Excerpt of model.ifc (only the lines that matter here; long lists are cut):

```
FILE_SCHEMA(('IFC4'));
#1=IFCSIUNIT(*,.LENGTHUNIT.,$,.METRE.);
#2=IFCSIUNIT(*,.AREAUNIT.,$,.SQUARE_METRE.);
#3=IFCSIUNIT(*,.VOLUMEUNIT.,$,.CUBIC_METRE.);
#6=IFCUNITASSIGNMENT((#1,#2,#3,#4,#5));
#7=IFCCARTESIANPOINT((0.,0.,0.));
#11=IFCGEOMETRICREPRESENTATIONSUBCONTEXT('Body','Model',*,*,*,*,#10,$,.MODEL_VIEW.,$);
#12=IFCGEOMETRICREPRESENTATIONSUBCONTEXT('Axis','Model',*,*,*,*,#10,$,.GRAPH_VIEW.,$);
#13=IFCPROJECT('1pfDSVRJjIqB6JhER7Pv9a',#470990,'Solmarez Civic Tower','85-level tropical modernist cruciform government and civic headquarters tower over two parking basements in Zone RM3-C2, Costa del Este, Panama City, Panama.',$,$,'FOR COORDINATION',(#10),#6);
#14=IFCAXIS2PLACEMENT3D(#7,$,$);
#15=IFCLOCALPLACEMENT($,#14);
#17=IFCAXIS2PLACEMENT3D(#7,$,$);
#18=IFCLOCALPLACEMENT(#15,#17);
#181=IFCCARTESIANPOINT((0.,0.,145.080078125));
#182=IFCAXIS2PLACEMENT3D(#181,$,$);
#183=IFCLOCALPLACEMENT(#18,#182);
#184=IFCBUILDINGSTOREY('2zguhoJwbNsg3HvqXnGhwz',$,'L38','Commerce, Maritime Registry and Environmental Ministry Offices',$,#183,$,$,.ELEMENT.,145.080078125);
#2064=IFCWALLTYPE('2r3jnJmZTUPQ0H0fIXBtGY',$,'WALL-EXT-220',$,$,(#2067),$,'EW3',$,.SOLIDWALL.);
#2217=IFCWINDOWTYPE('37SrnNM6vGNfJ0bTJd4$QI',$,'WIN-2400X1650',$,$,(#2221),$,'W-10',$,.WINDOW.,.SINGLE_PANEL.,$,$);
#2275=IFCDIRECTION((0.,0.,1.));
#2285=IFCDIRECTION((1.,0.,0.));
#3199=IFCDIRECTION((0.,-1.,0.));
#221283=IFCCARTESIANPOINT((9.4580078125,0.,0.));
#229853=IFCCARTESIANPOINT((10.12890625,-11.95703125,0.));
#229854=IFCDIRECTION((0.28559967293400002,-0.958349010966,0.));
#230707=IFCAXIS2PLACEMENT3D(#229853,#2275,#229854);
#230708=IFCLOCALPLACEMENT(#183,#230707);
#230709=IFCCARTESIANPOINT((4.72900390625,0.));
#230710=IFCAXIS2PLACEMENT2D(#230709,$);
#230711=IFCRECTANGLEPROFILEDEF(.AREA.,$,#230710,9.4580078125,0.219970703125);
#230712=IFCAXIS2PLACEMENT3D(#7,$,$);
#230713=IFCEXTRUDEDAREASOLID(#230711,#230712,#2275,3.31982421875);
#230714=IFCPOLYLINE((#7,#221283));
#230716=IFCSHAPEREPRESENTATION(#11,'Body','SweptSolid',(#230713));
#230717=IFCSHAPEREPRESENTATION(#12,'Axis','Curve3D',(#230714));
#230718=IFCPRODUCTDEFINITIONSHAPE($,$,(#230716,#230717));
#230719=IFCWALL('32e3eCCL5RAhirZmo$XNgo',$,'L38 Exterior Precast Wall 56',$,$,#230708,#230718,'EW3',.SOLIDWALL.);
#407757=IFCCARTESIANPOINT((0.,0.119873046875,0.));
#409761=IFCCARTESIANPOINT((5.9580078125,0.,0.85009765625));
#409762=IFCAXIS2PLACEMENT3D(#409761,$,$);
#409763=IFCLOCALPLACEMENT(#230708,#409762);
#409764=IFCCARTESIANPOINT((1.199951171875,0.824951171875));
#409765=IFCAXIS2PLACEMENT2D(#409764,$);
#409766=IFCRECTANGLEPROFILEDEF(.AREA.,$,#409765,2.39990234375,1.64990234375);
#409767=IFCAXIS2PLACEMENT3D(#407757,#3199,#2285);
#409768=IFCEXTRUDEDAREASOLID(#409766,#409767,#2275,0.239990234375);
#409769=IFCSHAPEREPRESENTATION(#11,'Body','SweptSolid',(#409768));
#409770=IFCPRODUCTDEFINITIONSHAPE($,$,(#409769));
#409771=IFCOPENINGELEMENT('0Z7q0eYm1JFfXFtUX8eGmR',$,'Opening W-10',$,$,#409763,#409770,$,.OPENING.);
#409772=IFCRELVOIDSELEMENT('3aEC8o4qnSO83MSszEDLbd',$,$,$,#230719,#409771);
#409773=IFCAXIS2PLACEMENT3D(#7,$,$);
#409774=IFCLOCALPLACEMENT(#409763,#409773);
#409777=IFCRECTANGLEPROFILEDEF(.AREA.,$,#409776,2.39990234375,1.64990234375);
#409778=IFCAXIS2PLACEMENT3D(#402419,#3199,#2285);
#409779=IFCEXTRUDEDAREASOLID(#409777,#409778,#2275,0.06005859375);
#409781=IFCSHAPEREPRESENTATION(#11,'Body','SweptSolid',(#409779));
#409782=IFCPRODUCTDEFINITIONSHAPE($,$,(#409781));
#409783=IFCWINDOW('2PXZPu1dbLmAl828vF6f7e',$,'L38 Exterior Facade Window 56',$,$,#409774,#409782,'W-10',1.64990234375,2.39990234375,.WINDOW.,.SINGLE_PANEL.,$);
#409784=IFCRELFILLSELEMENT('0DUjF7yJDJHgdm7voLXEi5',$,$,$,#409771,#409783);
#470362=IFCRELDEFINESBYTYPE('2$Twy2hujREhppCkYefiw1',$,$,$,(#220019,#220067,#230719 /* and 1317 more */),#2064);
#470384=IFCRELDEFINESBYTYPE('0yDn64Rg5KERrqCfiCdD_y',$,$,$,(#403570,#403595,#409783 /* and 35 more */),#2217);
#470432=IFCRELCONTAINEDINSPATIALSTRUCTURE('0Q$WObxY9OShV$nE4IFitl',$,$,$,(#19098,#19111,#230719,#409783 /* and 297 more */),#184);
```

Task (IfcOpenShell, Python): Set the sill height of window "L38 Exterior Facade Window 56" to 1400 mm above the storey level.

```python
import numpy as np
import ifcopenshell
import ifcopenshell.api.geometry
import ifcopenshell.geom
import ifcopenshell.util.element
import ifcopenshell.util.placement
import ifcopenshell.util.shape
import ifcopenshell.util.unit

model = ifcopenshell.open("model.ifc")
unit_scale = ifcopenshell.util.unit.calculate_unit_scale(model)

window = model.by_id(409783)
opening = window.FillsVoids[0].RelatingOpeningElement
storey = ifcopenshell.util.element.get_container(window, ifc_class="IfcBuildingStorey")
level = ifcopenshell.util.placement.get_local_placement(storey.ObjectPlacement)[2, 3]

# The opening's origin need not be at the sill, so measure its lowest point.
shape = ifcopenshell.geom.create_shape(ifcopenshell.geom.settings(), opening)
bottom = ifcopenshell.util.shape.get_shape_bottom_elevation(shape, shape.geometry) / unit_scale
dz = level + 1.4 / unit_scale - bottom

shift = np.array([0.0, 0.0, dz])
# The window is placed relative to its opening, so it follows when the opening moves.
matrix = ifcopenshell.util.placement.get_local_placement(opening.ObjectPlacement)
matrix[:3, 3] += shift
ifcopenshell.api.geometry.edit_object_placement(
    model, product=opening, matrix=matrix, is_si=False, should_transform_children=True
)

print(f"moved by {dz * unit_scale:+.3f} m")

model.write("model-out.ifc")
```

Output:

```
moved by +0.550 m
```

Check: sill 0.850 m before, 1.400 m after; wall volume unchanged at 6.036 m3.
